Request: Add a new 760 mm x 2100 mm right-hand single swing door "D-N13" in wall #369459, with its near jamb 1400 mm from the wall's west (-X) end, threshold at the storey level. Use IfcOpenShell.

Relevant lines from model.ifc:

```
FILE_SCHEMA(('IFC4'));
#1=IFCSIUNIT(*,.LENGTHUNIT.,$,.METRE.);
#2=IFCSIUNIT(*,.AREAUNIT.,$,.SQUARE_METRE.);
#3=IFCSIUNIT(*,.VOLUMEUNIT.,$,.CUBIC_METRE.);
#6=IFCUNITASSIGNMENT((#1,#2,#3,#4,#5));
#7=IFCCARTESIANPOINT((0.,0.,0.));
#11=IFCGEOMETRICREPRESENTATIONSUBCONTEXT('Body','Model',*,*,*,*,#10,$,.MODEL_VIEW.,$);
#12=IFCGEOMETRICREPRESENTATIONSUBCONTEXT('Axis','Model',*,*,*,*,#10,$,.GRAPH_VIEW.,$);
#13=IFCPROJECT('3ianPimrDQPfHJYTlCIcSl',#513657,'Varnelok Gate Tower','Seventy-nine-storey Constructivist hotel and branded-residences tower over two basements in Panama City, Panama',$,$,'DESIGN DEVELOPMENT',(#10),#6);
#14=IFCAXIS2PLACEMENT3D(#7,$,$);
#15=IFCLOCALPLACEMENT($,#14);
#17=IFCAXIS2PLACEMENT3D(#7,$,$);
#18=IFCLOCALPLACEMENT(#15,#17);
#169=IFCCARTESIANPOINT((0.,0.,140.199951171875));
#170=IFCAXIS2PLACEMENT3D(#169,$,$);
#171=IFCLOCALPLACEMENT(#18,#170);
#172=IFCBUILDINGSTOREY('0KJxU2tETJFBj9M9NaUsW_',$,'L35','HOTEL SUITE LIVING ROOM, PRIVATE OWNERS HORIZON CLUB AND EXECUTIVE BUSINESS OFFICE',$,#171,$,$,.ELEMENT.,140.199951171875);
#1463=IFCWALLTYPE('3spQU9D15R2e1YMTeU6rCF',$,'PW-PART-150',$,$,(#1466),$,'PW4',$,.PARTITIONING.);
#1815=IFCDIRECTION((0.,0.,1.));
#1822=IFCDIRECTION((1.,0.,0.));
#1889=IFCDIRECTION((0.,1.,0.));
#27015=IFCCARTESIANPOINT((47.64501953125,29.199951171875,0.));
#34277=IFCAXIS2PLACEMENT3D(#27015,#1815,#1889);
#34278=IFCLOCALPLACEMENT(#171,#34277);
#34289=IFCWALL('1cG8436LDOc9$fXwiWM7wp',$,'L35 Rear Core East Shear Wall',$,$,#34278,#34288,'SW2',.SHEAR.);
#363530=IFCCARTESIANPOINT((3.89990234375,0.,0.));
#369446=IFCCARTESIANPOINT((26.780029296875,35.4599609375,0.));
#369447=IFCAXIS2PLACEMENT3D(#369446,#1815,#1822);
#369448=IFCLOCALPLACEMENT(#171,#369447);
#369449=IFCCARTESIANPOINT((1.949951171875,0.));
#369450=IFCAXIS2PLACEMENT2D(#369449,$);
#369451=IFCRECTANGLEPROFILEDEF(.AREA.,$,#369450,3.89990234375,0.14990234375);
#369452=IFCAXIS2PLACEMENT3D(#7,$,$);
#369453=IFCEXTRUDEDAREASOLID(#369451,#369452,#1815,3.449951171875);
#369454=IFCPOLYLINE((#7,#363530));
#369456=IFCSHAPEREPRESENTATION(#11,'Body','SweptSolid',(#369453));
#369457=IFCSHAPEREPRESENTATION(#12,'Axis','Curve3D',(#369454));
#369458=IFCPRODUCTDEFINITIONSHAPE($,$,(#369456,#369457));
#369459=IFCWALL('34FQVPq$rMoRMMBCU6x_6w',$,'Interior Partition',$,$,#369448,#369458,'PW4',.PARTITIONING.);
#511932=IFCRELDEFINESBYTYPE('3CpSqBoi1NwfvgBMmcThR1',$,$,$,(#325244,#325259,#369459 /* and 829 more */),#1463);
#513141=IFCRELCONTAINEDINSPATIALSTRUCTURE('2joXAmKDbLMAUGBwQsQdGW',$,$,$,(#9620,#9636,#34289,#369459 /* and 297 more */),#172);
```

```python
import numpy as np
import ifcopenshell
import ifcopenshell.api.feature
import ifcopenshell.api.geometry
import ifcopenshell.api.root
import ifcopenshell.api.spatial
import ifcopenshell.geom
import ifcopenshell.util.element
import ifcopenshell.util.placement
import ifcopenshell.util.representation
import ifcopenshell.util.shape
import ifcopenshell.util.unit

model = ifcopenshell.open("model.ifc")
unit_scale = ifcopenshell.util.unit.calculate_unit_scale(model)
settings = ifcopenshell.geom.settings()


def volume(element):
    """Net volume in cubic metres, openings subtracted."""
    shape = ifcopenshell.geom.create_shape(settings, element)
    return ifcopenshell.util.shape.get_volume(shape.geometry)


wall = model.by_guid("34FQVPq$rMoRMMBCU6x_6w")
storey = ifcopenshell.util.element.get_container(wall, ifc_class="IfcBuildingStorey")
context = ifcopenshell.util.representation.get_context(model, "Model", "Body", "MODEL_VIEW")
before = volume(wall)

width, height, from_end, sill = 0.76, 2.1, 1.4, 0.0  # metres

# The wall runs along its own X axis, and the end named is its -X end.
wall_shape = ifcopenshell.geom.create_shape(settings, wall)
x, y, z = ifcopenshell.util.shape.get_vertices(wall_shape.geometry).T
start = x.min() + from_end
face, thickness = float(y.min()), float(y.max() - y.min())
wall_matrix = ifcopenshell.util.placement.get_local_placement(wall.ObjectPlacement)
level = ifcopenshell.util.placement.get_local_placement(storey.ObjectPlacement)[2, 3]


def in_wall(x, y):
    """Placement at x, y metres in the wall's axes, at sill height."""
    matrix = wall_matrix.copy()
    matrix[:, 3] = wall_matrix @ np.array([x / unit_scale, y / unit_scale, 0.0, 1.0])
    matrix[2, 3] = level + sill / unit_scale
    return matrix


# Opening: a box that overshoots both wall faces by 50 mm.
opening = ifcopenshell.api.root.create_entity(model, ifc_class="IfcOpeningElement", predefined_type="OPENING")
box = ifcopenshell.api.geometry.add_wall_representation(
    model, context=context, length=width, height=height, thickness=thickness + 0.1
)
ifcopenshell.api.geometry.assign_representation(model, product=opening, representation=box)
ifcopenshell.api.geometry.edit_object_placement(model, product=opening, matrix=in_wall(start, face - 0.05), is_si=False)
ifcopenshell.api.feature.add_feature(model, feature=opening, element=wall)

door = ifcopenshell.api.root.create_entity(model, ifc_class="IfcDoor", name="D-N13", predefined_type="DOOR")
door.OverallWidth, door.OverallHeight = width / unit_scale, height / unit_scale
door.OperationType = "SINGLE_SWING_RIGHT"
body = ifcopenshell.api.geometry.add_door_representation(
    model,
    context=context,
    overall_width=door.OverallWidth,
    overall_height=door.OverallHeight,
    operation_type="SINGLE_SWING_RIGHT",
    lining_properties={"LiningDepth": thickness / unit_scale, "ThresholdDepth": thickness / unit_scale},
)
ifcopenshell.api.geometry.assign_representation(model, product=door, representation=body)
ifcopenshell.api.spatial.assign_container(model, products=[door], relating_structure=storey)
ifcopenshell.api.feature.add_filling(model, opening=opening, element=door)

# The lining spans the wall, so the door starts at the wall face.
ifcopenshell.api.geometry.edit_object_placement(model, product=door, matrix=in_wall(start, face), is_si=False)

after = volume(wall)

print(f"wall volume {before:.3f} -> {after:.3f} m3")

model.write("model_rev.ifc")
```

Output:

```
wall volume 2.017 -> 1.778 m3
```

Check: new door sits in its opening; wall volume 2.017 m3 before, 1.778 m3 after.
